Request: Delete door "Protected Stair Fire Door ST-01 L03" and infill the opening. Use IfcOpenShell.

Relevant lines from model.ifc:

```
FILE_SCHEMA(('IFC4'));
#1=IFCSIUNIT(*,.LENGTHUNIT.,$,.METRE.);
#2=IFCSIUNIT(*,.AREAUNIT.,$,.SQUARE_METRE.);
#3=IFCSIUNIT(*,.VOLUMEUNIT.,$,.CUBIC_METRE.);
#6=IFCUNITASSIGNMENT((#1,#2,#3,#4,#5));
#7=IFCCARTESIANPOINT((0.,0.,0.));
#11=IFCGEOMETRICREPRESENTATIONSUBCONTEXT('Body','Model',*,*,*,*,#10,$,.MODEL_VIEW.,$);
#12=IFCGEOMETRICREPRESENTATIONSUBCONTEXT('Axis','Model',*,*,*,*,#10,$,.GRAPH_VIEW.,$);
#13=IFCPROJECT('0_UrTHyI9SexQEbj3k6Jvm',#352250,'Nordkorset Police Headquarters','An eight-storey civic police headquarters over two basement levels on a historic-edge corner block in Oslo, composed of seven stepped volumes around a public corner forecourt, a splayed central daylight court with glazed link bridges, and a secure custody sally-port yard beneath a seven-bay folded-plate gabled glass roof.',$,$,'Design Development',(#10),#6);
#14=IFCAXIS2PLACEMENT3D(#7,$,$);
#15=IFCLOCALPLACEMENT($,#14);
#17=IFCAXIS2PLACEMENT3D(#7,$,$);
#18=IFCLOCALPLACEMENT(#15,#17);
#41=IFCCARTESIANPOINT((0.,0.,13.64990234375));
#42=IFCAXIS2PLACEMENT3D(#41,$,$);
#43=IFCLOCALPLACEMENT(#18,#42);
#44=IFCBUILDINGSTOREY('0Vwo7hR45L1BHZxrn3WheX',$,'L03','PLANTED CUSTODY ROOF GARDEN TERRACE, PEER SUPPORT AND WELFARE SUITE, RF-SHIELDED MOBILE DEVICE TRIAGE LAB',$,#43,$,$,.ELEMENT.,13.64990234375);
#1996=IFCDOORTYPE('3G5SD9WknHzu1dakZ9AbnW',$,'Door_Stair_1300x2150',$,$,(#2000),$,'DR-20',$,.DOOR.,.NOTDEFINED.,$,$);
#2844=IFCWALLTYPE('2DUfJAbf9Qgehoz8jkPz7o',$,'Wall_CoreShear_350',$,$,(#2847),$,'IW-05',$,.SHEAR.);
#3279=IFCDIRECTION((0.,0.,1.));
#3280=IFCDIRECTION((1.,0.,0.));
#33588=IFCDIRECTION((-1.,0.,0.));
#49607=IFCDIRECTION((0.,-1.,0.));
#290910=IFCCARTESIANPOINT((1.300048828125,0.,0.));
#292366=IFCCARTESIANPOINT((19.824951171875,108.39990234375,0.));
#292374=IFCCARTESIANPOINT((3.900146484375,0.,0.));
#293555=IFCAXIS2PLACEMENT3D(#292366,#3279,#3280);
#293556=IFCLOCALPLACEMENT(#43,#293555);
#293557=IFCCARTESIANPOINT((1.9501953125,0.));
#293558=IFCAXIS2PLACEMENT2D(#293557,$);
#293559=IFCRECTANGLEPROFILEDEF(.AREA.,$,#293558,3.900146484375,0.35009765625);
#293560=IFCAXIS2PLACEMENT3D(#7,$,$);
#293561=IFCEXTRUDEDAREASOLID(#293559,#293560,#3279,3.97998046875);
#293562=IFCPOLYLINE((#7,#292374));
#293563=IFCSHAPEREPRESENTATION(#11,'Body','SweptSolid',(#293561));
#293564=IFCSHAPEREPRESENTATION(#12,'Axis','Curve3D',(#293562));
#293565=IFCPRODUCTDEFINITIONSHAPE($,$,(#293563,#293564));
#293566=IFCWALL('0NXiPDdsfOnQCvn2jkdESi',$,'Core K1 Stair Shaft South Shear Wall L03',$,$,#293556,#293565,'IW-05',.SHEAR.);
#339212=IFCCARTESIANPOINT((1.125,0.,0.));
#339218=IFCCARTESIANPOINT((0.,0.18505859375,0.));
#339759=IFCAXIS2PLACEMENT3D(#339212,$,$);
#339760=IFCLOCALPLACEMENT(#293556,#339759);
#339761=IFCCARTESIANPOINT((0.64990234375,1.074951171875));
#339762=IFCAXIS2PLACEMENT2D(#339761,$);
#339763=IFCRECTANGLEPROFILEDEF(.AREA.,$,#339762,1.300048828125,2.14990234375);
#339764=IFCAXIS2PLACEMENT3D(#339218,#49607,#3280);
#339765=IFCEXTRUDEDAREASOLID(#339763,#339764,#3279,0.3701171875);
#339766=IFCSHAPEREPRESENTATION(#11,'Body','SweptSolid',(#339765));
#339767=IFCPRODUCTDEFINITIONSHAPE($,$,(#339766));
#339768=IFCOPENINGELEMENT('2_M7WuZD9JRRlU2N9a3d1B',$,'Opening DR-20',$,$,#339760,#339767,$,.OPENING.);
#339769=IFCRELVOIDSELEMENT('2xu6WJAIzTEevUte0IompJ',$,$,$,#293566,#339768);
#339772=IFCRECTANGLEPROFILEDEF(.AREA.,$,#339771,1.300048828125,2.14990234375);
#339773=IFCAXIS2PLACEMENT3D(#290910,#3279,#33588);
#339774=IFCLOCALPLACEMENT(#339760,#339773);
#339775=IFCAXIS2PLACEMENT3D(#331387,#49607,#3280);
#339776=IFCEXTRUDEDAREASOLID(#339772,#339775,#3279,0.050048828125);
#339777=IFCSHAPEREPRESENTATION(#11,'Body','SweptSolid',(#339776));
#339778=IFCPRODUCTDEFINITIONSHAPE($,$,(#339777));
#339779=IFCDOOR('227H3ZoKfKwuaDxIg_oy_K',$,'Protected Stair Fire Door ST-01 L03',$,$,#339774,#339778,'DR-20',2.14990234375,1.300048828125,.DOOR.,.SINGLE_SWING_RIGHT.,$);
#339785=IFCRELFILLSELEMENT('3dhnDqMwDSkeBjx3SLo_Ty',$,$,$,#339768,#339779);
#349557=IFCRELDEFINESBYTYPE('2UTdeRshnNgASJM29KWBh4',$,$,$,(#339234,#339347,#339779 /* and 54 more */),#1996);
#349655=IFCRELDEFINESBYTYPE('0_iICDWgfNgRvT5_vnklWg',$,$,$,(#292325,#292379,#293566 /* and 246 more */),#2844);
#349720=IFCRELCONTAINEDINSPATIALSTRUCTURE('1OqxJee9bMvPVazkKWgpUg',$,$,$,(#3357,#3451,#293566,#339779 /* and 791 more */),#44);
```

```python
import ifcopenshell
import ifcopenshell.api.feature
import ifcopenshell.api.root
import ifcopenshell.geom
import ifcopenshell.util.shape

model = ifcopenshell.open("model.ifc")
settings = ifcopenshell.geom.settings()


def volume(element):
    """Net volume in cubic metres, openings subtracted."""
    shape = ifcopenshell.geom.create_shape(settings, element)
    return ifcopenshell.util.shape.get_volume(shape.geometry)


door = model.by_id(339779)
opening = door.FillsVoids[0].RelatingOpeningElement
wall = opening.VoidsElements[0].RelatingBuildingElement
before = volume(wall)

ifcopenshell.api.root.remove_product(model, product=door)
ifcopenshell.api.feature.remove_feature(model, feature=opening)

after = volume(wall)

print(f"wall volume {before:.3f} -> {after:.3f} m3")

model.write("model_rev.ifc")
```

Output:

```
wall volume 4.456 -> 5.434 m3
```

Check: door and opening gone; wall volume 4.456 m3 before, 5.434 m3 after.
